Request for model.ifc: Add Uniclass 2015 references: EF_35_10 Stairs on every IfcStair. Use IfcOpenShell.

First a look at what the model holds.

```python
import ifcopenshell

model = ifcopenshell.open("model.ifc")
print(model.schema)
print("classifications:", [c.Name for c in model.by_type("IfcClassification")])
for ifc_class in ("IfcDoor", "IfcRoof", "IfcStair", "IfcWall", "IfcWindow"):
    print(ifc_class, len(model.by_type(ifc_class)))
```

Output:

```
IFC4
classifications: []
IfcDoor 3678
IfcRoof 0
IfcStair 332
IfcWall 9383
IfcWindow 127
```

```python
import ifcopenshell
import ifcopenshell.api.classification

model = ifcopenshell.open("model.ifc")

system = ifcopenshell.api.classification.add_classification(model, classification="Uniclass 2015")

codes = {
    "IfcStair": ("EF_35_10", "Stairs"),
}
for ifc_class, (code, name) in codes.items():
    products = model.by_type(ifc_class)
    ifcopenshell.api.classification.add_reference(
        model, products=products, classification=system, identification=code, name=name
    )
    print(code, len(products))

model.write("model_edited.ifc")
```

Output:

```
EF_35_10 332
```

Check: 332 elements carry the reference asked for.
